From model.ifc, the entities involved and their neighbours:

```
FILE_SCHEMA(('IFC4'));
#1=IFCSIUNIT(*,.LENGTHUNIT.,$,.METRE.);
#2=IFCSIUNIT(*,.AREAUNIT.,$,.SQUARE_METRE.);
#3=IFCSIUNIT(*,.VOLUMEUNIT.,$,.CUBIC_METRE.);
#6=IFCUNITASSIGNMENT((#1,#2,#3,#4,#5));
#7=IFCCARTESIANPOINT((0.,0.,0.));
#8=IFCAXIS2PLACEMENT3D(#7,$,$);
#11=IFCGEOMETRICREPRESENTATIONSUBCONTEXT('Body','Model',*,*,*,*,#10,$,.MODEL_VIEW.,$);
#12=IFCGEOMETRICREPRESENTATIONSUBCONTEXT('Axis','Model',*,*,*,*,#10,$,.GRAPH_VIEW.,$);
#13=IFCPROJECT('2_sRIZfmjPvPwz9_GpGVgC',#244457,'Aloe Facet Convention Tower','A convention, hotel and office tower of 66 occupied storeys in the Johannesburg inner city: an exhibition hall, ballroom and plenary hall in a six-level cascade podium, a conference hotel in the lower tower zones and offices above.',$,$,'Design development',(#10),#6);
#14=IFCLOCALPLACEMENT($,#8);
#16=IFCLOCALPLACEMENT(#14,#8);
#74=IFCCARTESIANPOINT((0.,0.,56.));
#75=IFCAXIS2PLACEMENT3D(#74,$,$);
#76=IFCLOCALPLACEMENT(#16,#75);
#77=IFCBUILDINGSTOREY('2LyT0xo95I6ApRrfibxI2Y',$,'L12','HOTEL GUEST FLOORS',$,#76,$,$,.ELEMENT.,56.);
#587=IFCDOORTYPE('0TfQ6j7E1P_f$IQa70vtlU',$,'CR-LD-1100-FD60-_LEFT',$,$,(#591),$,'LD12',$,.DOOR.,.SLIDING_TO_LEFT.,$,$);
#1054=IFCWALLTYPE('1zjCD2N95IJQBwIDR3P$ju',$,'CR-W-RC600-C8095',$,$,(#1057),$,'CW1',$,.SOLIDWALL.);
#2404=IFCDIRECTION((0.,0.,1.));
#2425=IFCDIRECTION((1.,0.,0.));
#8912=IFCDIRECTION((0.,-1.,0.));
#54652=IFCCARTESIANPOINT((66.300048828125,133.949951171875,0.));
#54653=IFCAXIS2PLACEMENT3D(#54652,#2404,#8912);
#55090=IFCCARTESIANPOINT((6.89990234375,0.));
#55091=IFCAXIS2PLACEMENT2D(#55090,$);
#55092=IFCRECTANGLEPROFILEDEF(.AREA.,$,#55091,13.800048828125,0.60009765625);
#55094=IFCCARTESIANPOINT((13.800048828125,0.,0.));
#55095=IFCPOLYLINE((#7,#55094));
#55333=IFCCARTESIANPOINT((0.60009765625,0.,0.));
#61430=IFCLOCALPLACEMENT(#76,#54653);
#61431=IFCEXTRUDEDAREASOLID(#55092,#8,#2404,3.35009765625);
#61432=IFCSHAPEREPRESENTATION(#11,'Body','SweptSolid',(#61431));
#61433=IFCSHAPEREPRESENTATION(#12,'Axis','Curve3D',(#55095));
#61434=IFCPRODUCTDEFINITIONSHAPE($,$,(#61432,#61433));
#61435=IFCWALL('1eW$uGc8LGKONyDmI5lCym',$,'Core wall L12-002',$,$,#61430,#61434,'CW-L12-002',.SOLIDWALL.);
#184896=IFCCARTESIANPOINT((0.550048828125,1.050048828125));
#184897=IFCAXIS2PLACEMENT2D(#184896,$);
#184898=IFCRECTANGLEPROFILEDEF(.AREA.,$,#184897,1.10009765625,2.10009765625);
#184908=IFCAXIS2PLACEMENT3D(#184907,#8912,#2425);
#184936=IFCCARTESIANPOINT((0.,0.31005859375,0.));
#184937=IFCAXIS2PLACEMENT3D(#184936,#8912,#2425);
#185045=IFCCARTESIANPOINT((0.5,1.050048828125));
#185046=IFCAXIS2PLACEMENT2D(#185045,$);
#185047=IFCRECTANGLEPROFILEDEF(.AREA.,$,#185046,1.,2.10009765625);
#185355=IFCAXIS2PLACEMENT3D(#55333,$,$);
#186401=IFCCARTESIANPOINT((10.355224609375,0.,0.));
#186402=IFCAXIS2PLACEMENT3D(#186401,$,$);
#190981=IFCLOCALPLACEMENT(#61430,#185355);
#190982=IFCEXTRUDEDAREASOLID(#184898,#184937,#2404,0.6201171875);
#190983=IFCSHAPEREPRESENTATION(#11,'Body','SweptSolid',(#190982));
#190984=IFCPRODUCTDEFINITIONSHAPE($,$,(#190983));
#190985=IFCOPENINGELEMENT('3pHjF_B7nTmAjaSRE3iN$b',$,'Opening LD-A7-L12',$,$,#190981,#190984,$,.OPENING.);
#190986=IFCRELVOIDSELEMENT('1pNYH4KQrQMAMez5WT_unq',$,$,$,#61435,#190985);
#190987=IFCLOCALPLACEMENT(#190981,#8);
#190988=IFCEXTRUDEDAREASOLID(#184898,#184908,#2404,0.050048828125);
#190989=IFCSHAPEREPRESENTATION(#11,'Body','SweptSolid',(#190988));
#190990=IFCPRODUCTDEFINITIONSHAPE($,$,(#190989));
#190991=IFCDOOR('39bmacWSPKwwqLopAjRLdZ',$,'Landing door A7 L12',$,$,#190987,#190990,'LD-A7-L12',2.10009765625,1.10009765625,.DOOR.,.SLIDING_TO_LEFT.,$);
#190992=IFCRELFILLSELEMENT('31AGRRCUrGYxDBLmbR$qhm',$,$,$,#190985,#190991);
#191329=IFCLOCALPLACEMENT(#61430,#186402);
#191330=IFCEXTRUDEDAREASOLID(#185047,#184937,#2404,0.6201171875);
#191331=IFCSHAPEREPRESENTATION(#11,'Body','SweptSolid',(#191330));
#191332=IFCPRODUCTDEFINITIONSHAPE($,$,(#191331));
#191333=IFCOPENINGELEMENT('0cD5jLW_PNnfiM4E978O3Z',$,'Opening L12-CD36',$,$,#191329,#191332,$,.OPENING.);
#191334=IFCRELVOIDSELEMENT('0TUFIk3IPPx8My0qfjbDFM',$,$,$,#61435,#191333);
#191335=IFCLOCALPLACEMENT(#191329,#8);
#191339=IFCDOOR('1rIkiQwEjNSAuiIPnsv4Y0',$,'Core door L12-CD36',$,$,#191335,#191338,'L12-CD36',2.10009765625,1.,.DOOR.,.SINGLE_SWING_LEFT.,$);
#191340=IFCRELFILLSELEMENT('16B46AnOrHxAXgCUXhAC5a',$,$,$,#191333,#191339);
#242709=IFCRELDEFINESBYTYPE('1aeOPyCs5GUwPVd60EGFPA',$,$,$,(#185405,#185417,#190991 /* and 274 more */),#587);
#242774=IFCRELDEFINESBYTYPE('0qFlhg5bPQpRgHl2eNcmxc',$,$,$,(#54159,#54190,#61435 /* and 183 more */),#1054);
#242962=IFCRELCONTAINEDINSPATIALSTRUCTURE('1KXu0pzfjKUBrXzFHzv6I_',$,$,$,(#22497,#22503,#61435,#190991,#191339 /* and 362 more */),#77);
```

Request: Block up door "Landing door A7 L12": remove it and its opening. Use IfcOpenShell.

```python
import ifcopenshell
import ifcopenshell.api.feature
import ifcopenshell.api.root
import ifcopenshell.geom
import ifcopenshell.util.shape

model = ifcopenshell.open("model.ifc")
settings = ifcopenshell.geom.settings()


def volume(element):
    """Net volume in cubic metres, openings subtracted."""
    shape = ifcopenshell.geom.create_shape(settings, element)
    return ifcopenshell.util.shape.get_volume(shape.geometry)


door = model.by_guid("39bmacWSPKwwqLopAjRLdZ")
opening = door.FillsVoids[0].RelatingOpeningElement
wall = opening.VoidsElements[0].RelatingBuildingElement
before = volume(wall)

ifcopenshell.api.root.remove_product(model, product=door)
ifcopenshell.api.feature.remove_feature(model, feature=opening)

after = volume(wall)

print(f"wall volume {before:.3f} -> {after:.3f} m3")

model.write("model_updated.ifc")
```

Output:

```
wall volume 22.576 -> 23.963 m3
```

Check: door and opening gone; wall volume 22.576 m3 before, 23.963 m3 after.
